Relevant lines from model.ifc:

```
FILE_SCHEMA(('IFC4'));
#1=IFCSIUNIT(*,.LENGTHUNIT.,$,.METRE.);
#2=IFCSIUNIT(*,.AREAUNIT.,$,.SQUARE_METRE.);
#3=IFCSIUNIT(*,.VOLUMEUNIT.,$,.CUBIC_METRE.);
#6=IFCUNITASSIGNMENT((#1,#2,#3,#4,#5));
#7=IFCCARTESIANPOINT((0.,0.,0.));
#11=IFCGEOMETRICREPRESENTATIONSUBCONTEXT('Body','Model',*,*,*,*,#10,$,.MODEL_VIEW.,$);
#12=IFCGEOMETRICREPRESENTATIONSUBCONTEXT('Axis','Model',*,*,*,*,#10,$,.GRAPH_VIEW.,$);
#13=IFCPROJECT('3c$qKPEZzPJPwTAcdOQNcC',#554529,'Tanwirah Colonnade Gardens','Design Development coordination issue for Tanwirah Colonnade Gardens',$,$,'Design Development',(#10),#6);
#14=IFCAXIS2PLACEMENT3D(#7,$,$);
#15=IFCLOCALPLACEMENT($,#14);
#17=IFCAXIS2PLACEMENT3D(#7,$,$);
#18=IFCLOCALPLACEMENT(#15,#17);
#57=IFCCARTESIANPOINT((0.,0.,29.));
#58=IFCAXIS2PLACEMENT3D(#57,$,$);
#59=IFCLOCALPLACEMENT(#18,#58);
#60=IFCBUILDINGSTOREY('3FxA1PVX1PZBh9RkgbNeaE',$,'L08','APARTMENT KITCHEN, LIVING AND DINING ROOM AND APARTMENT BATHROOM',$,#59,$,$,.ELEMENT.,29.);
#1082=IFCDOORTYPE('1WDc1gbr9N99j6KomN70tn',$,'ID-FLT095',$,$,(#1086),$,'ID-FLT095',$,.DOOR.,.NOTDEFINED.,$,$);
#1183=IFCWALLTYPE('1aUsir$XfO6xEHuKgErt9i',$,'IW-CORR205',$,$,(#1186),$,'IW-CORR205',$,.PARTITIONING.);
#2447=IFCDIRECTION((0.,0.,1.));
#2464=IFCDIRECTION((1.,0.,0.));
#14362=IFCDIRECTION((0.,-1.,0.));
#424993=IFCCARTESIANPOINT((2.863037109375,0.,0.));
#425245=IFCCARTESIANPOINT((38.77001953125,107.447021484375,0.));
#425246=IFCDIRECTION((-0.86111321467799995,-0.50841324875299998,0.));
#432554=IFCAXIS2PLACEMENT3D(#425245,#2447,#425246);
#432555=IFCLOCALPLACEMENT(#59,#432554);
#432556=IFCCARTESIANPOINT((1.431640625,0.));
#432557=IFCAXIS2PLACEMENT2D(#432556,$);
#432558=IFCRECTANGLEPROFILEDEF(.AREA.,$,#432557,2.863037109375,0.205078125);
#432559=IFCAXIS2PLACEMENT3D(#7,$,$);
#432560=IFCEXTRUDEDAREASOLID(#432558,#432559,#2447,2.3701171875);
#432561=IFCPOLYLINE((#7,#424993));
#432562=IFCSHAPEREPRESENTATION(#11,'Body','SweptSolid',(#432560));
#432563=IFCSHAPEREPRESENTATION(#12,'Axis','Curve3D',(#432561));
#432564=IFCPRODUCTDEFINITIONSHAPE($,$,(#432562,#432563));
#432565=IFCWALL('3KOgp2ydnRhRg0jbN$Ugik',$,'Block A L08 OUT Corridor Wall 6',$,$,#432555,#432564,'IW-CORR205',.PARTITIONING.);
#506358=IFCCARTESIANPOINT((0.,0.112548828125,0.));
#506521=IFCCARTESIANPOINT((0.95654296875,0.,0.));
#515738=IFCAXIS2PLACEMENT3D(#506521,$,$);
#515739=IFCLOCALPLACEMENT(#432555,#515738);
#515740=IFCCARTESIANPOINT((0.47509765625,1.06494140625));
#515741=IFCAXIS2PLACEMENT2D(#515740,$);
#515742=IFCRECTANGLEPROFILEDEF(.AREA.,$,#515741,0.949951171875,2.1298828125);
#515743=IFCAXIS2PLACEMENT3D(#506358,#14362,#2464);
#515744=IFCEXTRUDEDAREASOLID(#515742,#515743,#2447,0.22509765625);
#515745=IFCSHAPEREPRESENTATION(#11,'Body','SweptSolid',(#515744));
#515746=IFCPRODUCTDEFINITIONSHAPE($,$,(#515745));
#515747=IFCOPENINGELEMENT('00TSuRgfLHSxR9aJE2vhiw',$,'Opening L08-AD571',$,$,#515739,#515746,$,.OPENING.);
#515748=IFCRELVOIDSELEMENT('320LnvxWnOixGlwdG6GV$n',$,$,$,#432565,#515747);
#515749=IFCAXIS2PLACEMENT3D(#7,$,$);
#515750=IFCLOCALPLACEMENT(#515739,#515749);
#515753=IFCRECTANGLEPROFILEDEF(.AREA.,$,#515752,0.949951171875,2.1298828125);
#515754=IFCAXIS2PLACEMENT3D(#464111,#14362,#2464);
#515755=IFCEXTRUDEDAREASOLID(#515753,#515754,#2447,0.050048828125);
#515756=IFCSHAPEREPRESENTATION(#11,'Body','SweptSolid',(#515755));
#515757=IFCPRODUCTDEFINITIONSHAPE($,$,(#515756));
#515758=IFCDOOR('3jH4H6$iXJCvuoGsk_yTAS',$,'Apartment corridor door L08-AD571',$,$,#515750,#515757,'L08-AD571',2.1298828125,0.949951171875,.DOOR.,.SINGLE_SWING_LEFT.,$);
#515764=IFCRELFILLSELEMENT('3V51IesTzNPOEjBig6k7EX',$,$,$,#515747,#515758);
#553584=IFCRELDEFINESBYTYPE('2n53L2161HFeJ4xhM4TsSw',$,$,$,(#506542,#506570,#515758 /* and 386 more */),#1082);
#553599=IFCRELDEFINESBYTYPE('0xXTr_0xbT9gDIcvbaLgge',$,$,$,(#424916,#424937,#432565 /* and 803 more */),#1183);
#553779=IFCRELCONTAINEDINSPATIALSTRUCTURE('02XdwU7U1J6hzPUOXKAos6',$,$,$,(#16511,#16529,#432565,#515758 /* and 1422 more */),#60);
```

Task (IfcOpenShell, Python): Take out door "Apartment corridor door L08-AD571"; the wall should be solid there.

```python
import ifcopenshell
import ifcopenshell.api.feature
import ifcopenshell.api.root
import ifcopenshell.geom
import ifcopenshell.util.shape

model = ifcopenshell.open("model.ifc")
settings = ifcopenshell.geom.settings()


def volume(element):
    """Net volume in cubic metres, openings subtracted."""
    shape = ifcopenshell.geom.create_shape(settings, element)
    return ifcopenshell.util.shape.get_volume(shape.geometry)


door = model.by_guid("3jH4H6$iXJCvuoGsk_yTAS")
opening = door.FillsVoids[0].RelatingOpeningElement
wall = opening.VoidsElements[0].RelatingBuildingElement
before = volume(wall)

ifcopenshell.api.root.remove_product(model, product=door)
ifcopenshell.api.feature.remove_feature(model, feature=opening)

after = volume(wall)

print(f"wall volume {before:.3f} -> {after:.3f} m3")

model.write("model_edited.ifc")
```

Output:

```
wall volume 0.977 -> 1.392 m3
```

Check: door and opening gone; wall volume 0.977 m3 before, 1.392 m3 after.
